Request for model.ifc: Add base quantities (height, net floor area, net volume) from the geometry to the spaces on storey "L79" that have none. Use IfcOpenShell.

First a look at what the model holds.

```python
import ifcopenshell
import ifcopenshell.util.element
import ifcopenshell.util.unit

model = ifcopenshell.open("model.ifc")
print(model.schema)
for unit_type in ("LENGTHUNIT", "AREAUNIT", "VOLUMEUNIT"):
    print(unit_type, ifcopenshell.util.unit.calculate_unit_scale(model, unit_type))
storey = next(s for s in model.by_type("IfcBuildingStorey") if s.Name == "L79")
spaces = [e for e in ifcopenshell.util.element.get_decomposition(storey) if e.is_a("IfcSpace")]
for e in sorted(spaces, key=lambda e: e.id()):
    print(e.id(), e.is_a(), e.Name, list(ifcopenshell.util.element.get_psets(e, qtos_only=True)), sep=" | ")
```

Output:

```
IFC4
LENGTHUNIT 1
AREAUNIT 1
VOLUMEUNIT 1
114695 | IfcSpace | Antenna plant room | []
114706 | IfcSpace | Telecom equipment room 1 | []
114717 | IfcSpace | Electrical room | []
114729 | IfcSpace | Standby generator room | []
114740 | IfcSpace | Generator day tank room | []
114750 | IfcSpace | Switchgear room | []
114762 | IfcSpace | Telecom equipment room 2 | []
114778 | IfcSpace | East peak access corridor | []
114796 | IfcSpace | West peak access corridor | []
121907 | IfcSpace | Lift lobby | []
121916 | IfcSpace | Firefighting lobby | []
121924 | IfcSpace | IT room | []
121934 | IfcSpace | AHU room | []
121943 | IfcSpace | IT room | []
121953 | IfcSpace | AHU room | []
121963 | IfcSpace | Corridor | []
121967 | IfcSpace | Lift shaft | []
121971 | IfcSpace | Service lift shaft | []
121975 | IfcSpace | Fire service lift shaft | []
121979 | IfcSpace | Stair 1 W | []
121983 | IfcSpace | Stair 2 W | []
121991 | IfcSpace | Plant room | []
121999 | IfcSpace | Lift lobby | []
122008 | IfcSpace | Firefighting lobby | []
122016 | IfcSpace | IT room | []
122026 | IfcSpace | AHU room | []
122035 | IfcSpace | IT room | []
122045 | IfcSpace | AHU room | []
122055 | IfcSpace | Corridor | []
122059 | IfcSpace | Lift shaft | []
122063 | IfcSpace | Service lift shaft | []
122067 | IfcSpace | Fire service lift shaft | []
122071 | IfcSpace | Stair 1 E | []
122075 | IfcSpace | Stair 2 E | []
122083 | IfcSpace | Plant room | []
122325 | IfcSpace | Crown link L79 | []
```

```python
import ifcopenshell
import ifcopenshell.api.pset
import ifcopenshell.geom
import ifcopenshell.util.element
import ifcopenshell.util.shape
import ifcopenshell.util.unit

model = ifcopenshell.open("model.ifc")
unit_scale = ifcopenshell.util.unit.calculate_unit_scale(model)
area_scale = ifcopenshell.util.unit.calculate_unit_scale(model, "AREAUNIT")
volume_scale = ifcopenshell.util.unit.calculate_unit_scale(model, "VOLUMEUNIT")
settings = ifcopenshell.geom.settings()

storey = next(s for s in model.by_type("IfcBuildingStorey") if s.Name == "L79")
spaces = [e for e in ifcopenshell.util.element.get_decomposition(storey) if e.is_a("IfcSpace")]

for e in sorted(spaces, key=lambda e: e.id()):
    if ifcopenshell.util.element.get_psets(e, qtos_only=True, should_inherit=False):
        continue
    # Geometry comes back in metres, in the element's own axes.
    shape = ifcopenshell.geom.create_shape(settings, e)
    values = {
        "Height": ifcopenshell.util.shape.get_z(shape.geometry) / unit_scale,
        "NetFloorArea": ifcopenshell.util.shape.get_footprint_area(shape.geometry) / area_scale,
        "NetVolume": ifcopenshell.util.shape.get_volume(shape.geometry) / volume_scale,
    }
    qto = ifcopenshell.api.pset.add_qto(model, product=e, name="Qto_SpaceBaseQuantities")
    ifcopenshell.api.pset.edit_qto(model, qto=qto, properties=values)
    print(e.id(), {k: round(v, 3) for k, v in values.items()})

model.write("model_edited.ifc")
```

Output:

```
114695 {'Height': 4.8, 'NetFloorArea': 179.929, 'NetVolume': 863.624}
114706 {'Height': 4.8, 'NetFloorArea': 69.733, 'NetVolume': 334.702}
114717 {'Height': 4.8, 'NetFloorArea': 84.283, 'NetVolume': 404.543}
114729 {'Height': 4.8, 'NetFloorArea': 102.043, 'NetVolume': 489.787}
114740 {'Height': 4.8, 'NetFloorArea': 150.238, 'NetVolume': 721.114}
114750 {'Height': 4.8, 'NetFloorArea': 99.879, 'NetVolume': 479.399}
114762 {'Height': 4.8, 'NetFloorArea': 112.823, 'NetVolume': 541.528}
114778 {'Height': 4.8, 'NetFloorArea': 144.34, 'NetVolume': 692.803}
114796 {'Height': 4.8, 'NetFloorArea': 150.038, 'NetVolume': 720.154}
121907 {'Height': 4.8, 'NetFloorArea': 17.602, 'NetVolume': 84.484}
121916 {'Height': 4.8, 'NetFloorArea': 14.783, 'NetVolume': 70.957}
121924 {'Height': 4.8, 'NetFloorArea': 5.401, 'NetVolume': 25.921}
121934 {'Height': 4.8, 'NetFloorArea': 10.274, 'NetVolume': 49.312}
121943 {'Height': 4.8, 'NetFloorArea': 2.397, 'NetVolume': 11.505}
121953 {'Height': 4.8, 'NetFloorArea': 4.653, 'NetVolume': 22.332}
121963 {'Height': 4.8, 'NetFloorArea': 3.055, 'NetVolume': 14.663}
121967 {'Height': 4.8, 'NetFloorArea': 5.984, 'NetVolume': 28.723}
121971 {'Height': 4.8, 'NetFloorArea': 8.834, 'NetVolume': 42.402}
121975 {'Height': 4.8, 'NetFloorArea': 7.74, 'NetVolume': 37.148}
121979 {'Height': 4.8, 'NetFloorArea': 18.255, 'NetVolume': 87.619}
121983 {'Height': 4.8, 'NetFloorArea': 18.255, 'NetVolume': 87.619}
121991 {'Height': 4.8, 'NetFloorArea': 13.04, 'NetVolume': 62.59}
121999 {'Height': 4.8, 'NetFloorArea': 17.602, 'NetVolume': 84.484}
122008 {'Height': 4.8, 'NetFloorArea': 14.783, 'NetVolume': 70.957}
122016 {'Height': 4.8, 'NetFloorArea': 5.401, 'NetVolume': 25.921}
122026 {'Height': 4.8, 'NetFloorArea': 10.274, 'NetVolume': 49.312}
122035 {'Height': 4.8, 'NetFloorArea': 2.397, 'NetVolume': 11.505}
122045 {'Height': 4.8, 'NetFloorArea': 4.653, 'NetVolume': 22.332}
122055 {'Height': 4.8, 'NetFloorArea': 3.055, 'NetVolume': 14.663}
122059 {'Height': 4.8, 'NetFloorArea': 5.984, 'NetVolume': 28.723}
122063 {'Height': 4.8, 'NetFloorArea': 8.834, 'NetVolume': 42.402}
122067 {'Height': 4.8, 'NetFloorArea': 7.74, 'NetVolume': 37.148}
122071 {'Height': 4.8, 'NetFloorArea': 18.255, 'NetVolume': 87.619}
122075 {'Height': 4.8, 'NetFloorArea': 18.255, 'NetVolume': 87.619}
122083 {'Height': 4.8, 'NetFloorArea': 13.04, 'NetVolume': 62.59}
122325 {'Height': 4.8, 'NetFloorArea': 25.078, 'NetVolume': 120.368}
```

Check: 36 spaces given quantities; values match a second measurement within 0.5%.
